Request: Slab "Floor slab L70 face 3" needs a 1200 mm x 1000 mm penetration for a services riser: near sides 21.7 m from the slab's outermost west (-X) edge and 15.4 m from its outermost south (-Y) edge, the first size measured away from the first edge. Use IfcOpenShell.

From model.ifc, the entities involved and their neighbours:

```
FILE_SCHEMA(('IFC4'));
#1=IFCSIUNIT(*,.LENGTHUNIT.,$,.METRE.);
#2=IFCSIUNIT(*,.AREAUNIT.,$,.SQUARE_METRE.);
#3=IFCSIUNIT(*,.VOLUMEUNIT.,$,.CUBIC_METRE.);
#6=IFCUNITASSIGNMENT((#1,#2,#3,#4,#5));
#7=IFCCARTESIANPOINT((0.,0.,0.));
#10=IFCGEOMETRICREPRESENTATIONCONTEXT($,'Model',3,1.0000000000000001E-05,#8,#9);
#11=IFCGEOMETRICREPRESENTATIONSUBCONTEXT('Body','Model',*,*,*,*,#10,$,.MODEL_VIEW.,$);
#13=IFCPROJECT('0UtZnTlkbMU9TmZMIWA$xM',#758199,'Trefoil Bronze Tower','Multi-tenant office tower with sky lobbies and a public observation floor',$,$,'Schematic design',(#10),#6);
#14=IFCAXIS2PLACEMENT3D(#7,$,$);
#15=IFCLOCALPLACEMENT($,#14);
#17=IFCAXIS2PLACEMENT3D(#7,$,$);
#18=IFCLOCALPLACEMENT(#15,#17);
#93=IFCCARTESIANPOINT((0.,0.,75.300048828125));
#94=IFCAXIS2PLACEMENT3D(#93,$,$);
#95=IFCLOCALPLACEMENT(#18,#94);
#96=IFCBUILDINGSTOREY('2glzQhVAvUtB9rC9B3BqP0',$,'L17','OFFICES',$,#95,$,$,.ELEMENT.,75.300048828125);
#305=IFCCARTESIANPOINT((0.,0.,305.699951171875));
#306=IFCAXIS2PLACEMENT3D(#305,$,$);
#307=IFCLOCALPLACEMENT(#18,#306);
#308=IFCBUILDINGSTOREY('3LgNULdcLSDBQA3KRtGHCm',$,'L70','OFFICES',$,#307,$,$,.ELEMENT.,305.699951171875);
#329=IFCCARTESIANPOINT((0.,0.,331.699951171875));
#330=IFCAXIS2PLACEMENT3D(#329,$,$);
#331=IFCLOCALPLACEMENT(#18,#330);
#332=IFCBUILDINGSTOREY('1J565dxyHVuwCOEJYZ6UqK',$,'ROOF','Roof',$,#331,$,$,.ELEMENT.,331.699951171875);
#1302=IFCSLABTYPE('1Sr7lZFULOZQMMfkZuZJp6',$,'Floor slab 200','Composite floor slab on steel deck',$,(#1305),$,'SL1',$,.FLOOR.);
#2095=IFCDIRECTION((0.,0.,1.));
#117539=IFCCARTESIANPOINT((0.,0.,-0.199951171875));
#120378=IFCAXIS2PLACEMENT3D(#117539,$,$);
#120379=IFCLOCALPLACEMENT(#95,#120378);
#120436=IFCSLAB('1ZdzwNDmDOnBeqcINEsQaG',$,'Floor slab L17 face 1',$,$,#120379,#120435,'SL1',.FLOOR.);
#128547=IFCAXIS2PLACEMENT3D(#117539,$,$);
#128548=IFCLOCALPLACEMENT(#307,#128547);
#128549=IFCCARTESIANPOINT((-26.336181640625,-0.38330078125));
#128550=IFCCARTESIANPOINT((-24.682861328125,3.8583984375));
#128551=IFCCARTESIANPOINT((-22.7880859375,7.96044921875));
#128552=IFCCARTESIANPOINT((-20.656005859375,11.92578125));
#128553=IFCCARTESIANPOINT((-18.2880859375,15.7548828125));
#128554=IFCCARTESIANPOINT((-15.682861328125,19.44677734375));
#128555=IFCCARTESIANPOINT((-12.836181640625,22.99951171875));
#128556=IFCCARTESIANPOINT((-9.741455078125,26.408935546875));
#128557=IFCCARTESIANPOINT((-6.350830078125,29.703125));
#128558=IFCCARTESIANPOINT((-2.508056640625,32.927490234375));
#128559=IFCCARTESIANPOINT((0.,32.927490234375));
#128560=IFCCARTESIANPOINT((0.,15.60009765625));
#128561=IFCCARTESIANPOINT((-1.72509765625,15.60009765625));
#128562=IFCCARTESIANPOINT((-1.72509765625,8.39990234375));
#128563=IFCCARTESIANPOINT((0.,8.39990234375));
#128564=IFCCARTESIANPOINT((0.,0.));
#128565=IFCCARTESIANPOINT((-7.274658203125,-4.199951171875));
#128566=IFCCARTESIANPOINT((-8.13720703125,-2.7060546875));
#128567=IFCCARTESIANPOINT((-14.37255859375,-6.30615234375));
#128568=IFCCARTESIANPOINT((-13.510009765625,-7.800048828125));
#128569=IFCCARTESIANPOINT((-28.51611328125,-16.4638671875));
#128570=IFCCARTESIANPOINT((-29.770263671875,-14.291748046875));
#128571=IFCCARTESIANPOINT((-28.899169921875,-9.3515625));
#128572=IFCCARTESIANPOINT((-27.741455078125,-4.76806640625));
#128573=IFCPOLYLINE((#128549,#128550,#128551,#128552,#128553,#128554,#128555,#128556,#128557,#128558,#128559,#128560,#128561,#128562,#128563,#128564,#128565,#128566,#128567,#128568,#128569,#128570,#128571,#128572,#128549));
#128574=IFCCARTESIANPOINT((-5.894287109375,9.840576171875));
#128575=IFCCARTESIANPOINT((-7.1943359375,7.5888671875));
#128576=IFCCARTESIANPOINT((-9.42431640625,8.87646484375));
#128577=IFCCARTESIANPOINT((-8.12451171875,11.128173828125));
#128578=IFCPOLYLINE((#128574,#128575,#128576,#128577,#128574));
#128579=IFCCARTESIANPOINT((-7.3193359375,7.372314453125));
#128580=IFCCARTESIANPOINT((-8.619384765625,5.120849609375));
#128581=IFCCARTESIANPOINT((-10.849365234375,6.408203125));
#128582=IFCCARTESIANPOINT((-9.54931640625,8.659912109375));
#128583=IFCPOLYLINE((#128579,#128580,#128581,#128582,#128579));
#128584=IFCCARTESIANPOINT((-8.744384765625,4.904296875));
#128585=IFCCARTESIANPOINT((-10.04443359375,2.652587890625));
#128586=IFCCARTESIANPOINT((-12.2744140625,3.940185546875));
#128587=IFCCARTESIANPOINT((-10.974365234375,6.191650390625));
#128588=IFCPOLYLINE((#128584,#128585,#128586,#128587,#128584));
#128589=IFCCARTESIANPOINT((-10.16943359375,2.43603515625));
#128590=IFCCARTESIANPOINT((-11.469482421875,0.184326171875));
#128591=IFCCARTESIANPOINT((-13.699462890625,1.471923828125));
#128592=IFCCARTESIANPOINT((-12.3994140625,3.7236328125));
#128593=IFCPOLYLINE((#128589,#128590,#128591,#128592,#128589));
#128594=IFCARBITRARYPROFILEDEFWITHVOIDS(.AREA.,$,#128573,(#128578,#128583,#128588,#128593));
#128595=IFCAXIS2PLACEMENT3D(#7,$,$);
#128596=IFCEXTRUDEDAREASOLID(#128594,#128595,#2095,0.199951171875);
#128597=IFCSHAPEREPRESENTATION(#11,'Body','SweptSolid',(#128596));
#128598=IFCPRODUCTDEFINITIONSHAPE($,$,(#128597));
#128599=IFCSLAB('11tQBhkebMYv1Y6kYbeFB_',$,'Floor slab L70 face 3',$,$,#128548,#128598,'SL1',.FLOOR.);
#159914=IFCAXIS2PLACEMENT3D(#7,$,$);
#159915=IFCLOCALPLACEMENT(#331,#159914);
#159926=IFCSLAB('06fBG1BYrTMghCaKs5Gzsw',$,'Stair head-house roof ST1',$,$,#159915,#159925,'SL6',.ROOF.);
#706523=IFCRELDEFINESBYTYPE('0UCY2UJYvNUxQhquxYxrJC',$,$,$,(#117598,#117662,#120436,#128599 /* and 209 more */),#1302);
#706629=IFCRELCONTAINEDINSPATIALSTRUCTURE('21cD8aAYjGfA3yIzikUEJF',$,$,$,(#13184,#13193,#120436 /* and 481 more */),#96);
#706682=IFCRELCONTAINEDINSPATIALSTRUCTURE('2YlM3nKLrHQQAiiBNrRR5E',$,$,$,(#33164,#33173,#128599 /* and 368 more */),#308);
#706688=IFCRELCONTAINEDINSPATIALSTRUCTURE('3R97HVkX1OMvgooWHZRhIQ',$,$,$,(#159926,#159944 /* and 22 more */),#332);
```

```python
import numpy as np
import ifcopenshell
import ifcopenshell.api.feature
import ifcopenshell.api.geometry
import ifcopenshell.api.root
import ifcopenshell.geom
import ifcopenshell.util.placement
import ifcopenshell.util.representation
import ifcopenshell.util.shape
import ifcopenshell.util.unit

model = ifcopenshell.open("model.ifc")
unit_scale = ifcopenshell.util.unit.calculate_unit_scale(model)
settings = ifcopenshell.geom.settings()


def volume(element):
    """Net volume in cubic metres, openings subtracted."""
    shape = ifcopenshell.geom.create_shape(settings, element)
    return ifcopenshell.util.shape.get_volume(shape.geometry)


slab = model.by_guid("11tQBhkebMYv1Y6kYbeFB_")
before = volume(slab)

# Extent in the slab's own axes, in metres. The edges named are its -X and -Y sides.
slab_shape = ifcopenshell.geom.create_shape(settings, slab)
vertices = ifcopenshell.util.shape.get_vertices(slab_shape.geometry)
x_min, y_min, bottom = vertices.min(axis=0)
top = vertices[:, 2].max()

opening = ifcopenshell.api.root.create_entity(model, ifc_class="IfcOpeningElement", name="Services riser opening", predefined_type="OPENING")
context = ifcopenshell.util.representation.get_context(model, "Model", "Body", "MODEL_VIEW")
width, depth = 1.2, 1
outline = [(0.0, 0.0), (width, 0.0), (width, depth), (0.0, depth), (0.0, 0.0)]
# Overshoot both faces by 50 mm so the cut is clean.
shape = ifcopenshell.api.geometry.add_slab_representation(
    model, context=context, depth=top - bottom + 0.1, polyline=outline
)
ifcopenshell.api.geometry.assign_representation(model, product=opening, representation=shape)

matrix = ifcopenshell.util.placement.get_local_placement(slab.ObjectPlacement)
matrix[:, 3] = matrix @ np.append(np.array([x_min + 21.7, y_min + 15.4, bottom - 0.05]) / unit_scale, 1.0)
ifcopenshell.api.geometry.edit_object_placement(model, product=opening, matrix=matrix, is_si=False)
ifcopenshell.api.feature.add_feature(model, feature=opening, element=slab)

after = volume(slab)

print(f"slab volume {before:.3f} -> {after:.3f} m3")

model.write("model_rev.ifc")
```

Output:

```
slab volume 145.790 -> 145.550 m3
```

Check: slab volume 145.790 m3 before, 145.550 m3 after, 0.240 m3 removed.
